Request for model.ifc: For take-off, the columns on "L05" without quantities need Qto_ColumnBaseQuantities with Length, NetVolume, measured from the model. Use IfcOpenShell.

First a look at what the model holds.

```python
import ifcopenshell
import ifcopenshell.util.element
import ifcopenshell.util.unit

model = ifcopenshell.open("model.ifc")
print(model.schema)
for unit_type in ("LENGTHUNIT", "AREAUNIT", "VOLUMEUNIT"):
    print(unit_type, ifcopenshell.util.unit.calculate_unit_scale(model, unit_type))
storey = next(s for s in model.by_type("IfcBuildingStorey") if s.Name == "L05")
columns = [e for e in ifcopenshell.util.element.get_decomposition(storey) if e.is_a("IfcColumn")]
for e in sorted(columns, key=lambda e: e.id()):
    print(e.id(), e.is_a(), e.Name, list(ifcopenshell.util.element.get_psets(e, qtos_only=True)), sep=" | ")
```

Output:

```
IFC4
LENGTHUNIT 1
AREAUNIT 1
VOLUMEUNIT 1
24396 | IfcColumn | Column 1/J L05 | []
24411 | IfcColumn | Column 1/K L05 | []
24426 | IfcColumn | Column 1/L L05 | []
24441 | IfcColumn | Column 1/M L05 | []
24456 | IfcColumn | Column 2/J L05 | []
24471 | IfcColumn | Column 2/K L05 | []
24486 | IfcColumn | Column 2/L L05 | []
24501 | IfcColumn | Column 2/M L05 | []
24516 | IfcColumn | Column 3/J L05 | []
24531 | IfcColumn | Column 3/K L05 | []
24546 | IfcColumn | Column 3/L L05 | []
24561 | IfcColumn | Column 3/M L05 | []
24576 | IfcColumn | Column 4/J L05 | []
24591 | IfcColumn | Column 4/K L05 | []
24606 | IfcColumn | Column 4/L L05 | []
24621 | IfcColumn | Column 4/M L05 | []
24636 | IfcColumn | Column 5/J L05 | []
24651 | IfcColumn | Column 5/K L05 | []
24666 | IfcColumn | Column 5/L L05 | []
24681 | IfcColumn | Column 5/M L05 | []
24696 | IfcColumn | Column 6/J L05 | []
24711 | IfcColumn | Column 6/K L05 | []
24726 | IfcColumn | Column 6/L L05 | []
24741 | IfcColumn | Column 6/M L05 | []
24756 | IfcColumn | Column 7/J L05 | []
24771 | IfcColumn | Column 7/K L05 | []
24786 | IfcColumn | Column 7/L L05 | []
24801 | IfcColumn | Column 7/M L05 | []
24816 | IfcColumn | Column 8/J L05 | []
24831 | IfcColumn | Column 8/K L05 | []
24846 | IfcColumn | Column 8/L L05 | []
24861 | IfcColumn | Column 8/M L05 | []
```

```python
import ifcopenshell
import ifcopenshell.api.pset
import ifcopenshell.geom
import ifcopenshell.util.element
import ifcopenshell.util.shape
import ifcopenshell.util.unit

model = ifcopenshell.open("model.ifc")
unit_scale = ifcopenshell.util.unit.calculate_unit_scale(model)
volume_scale = ifcopenshell.util.unit.calculate_unit_scale(model, "VOLUMEUNIT")
settings = ifcopenshell.geom.settings()

storey = next(s for s in model.by_type("IfcBuildingStorey") if s.Name == "L05")
columns = [e for e in ifcopenshell.util.element.get_decomposition(storey) if e.is_a("IfcColumn")]

for e in sorted(columns, key=lambda e: e.id()):
    if ifcopenshell.util.element.get_psets(e, qtos_only=True, should_inherit=False):
        continue
    # Geometry comes back in metres, in the element's own axes.
    shape = ifcopenshell.geom.create_shape(settings, e)
    values = {
        "Length": ifcopenshell.util.shape.get_z(shape.geometry) / unit_scale,
        "NetVolume": ifcopenshell.util.shape.get_volume(shape.geometry) / volume_scale,
    }
    qto = ifcopenshell.api.pset.add_qto(model, product=e, name="Qto_ColumnBaseQuantities")
    ifcopenshell.api.pset.edit_qto(model, qto=qto, properties=values)
    print(e.id(), {k: round(v, 3) for k, v in values.items()})

model.write("model-out.ifc")
```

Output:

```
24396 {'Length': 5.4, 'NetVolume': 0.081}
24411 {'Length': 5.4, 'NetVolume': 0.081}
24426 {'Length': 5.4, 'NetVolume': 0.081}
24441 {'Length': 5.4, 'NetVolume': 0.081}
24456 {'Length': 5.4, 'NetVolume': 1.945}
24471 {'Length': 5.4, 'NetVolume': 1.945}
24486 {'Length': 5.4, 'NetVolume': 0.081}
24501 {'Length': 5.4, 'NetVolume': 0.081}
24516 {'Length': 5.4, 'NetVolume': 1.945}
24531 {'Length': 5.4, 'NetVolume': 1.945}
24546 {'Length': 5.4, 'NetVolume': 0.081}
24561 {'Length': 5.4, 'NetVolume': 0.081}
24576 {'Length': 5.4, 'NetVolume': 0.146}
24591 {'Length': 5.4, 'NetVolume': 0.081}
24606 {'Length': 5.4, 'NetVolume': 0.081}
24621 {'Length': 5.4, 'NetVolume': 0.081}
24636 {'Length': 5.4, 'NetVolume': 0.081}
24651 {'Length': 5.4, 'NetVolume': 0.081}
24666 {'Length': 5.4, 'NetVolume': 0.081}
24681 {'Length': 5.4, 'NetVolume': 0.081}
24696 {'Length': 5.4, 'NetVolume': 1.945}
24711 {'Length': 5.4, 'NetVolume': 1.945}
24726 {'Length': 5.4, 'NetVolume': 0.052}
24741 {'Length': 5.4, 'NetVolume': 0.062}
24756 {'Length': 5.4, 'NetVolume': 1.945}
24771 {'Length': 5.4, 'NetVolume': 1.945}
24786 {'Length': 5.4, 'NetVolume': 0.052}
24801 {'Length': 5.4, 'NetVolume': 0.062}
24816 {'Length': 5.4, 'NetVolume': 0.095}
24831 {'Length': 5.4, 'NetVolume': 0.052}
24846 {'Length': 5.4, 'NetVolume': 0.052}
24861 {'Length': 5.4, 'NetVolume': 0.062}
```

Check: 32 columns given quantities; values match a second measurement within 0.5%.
